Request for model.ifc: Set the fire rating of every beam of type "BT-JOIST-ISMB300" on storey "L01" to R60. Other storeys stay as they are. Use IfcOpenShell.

First a look at what the model holds.

```python
import ifcopenshell
import ifcopenshell.util.element

model = ifcopenshell.open("model.ifc")
print(model.schema)
storey = next(s for s in model.by_type("IfcBuildingStorey") if s.Name == "L01")
beams = [e for e in ifcopenshell.util.element.get_decomposition(storey) if e.is_a("IfcBeam")]
seen = {}
for e in beams:
    element_type = ifcopenshell.util.element.get_type(e)
    key = (element_type.Name if element_type != e and element_type else None, ifcopenshell.util.element.get_pset(e, "Pset_BeamCommon", "FireRating"))
    seen[key] = seen.get(key, 0) + 1
for (name, value), count in sorted(seen.items(), key=str):
    print(count, "x", name, "|", value)
```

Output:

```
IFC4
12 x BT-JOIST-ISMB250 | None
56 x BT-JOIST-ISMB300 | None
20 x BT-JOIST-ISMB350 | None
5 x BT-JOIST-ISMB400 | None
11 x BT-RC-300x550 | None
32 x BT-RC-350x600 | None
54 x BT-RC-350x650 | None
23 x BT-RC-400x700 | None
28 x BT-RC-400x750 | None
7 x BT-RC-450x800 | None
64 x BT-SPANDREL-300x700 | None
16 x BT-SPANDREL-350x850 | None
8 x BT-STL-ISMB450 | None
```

```python
import ifcopenshell
import ifcopenshell.api.pset
import ifcopenshell.util.element

model = ifcopenshell.open("model.ifc")

storey = next(s for s in model.by_type("IfcBuildingStorey") if s.Name == "L01")
beams = [e for e in ifcopenshell.util.element.get_decomposition(storey) if e.is_a("IfcBeam")]

count = 0
for e in beams:
    element_type = ifcopenshell.util.element.get_type(e)
    if element_type in (None, e) or element_type.Name != "BT-JOIST-ISMB300":
        continue
    # add_pset returns the element's existing set when there is one.
    pset = ifcopenshell.api.pset.add_pset(model, product=e, name="Pset_BeamCommon")
    ifcopenshell.api.pset.edit_pset(model, pset=pset, properties={"FireRating": "R60"})
    count += 1

print(count, "beams updated")

model.write("model_v2.ifc")
```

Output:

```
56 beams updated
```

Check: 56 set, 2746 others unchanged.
